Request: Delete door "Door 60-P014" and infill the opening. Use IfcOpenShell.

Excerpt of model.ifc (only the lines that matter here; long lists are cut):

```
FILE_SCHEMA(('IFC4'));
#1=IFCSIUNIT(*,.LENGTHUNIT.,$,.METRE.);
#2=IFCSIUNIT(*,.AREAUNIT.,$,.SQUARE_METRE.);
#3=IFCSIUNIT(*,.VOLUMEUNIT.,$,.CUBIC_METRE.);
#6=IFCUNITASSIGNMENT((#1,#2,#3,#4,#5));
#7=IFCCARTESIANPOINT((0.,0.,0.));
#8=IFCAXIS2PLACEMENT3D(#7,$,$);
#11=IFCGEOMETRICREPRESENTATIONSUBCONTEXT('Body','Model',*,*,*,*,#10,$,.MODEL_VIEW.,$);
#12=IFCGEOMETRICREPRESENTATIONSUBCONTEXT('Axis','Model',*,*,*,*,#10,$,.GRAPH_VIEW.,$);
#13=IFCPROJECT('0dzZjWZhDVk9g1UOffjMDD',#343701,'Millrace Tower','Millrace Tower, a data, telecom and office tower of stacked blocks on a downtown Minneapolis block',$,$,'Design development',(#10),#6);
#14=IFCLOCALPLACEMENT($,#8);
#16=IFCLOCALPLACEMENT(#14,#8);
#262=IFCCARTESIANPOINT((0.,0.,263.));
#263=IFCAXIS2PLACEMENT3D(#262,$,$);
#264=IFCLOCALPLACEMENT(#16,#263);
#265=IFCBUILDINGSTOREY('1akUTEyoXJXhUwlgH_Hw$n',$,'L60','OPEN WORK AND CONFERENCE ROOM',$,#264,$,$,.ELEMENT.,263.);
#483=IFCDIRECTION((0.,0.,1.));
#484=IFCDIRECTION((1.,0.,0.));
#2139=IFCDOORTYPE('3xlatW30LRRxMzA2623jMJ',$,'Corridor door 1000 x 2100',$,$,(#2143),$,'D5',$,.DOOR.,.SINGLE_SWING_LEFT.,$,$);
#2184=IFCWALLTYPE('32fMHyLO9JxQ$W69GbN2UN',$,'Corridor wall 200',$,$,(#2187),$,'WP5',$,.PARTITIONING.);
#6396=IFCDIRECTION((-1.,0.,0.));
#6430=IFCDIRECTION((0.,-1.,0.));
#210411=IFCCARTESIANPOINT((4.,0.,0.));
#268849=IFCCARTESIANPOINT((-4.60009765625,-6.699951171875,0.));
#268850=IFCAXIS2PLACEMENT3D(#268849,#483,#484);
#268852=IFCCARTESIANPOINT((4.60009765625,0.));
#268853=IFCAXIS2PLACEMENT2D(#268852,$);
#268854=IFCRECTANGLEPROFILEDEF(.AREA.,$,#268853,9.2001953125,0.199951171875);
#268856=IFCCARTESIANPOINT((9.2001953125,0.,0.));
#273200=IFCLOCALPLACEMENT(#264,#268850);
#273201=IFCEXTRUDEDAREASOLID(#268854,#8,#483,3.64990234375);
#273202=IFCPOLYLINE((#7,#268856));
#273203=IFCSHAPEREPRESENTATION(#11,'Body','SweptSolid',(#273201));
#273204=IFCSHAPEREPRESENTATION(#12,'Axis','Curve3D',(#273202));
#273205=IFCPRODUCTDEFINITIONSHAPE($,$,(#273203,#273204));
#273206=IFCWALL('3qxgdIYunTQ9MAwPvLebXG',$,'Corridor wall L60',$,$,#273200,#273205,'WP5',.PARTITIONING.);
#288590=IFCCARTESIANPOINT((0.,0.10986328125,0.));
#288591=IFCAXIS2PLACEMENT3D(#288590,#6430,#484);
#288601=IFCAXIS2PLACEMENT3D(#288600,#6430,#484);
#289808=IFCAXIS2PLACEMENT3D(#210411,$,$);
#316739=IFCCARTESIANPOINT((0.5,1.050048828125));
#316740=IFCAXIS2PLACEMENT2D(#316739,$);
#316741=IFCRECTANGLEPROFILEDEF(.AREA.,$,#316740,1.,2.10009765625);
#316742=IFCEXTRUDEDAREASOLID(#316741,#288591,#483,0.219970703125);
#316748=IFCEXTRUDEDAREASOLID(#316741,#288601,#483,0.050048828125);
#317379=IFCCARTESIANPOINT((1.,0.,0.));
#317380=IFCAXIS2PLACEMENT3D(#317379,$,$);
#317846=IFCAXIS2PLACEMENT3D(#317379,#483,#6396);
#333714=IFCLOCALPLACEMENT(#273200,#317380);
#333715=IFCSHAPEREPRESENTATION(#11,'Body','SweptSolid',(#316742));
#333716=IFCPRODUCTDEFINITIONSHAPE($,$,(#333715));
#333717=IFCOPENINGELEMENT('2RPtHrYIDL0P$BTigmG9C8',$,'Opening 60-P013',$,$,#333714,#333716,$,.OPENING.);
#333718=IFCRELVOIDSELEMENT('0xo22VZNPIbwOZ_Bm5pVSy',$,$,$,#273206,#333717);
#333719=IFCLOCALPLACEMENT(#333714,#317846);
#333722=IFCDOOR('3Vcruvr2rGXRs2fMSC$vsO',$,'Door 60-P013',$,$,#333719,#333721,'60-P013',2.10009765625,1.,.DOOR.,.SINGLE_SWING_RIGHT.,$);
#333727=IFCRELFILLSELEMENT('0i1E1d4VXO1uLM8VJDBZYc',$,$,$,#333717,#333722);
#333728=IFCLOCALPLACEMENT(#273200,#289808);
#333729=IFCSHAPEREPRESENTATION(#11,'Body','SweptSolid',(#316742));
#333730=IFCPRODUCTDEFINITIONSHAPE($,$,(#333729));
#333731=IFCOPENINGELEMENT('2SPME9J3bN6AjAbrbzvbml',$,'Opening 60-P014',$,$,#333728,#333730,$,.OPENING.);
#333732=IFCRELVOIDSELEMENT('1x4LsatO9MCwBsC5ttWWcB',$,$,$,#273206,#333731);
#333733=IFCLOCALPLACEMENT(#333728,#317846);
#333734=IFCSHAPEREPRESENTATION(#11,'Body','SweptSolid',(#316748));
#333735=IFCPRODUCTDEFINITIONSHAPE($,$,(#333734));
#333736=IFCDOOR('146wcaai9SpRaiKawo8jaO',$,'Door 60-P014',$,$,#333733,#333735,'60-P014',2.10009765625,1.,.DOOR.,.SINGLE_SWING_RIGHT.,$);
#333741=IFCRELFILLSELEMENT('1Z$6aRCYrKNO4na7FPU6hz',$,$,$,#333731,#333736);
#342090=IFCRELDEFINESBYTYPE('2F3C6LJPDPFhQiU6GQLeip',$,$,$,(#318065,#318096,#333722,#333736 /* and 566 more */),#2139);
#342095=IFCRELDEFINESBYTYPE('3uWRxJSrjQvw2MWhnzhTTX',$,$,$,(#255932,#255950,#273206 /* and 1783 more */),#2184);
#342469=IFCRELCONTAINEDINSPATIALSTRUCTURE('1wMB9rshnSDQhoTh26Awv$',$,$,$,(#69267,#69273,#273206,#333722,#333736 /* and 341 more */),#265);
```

```python
import ifcopenshell
import ifcopenshell.api.feature
import ifcopenshell.api.root
import ifcopenshell.geom
import ifcopenshell.util.shape

model = ifcopenshell.open("model.ifc")
settings = ifcopenshell.geom.settings()


def volume(element):
    """Net volume in cubic metres, openings subtracted."""
    shape = ifcopenshell.geom.create_shape(settings, element)
    return ifcopenshell.util.shape.get_volume(shape.geometry)


door = model.by_id(333736)
opening = door.FillsVoids[0].RelatingOpeningElement
wall = opening.VoidsElements[0].RelatingBuildingElement
before = volume(wall)

ifcopenshell.api.root.remove_product(model, product=door)
ifcopenshell.api.feature.remove_feature(model, feature=opening)

after = volume(wall)

print(f"wall volume {before:.3f} -> {after:.3f} m3")

model.write("model-out.ifc")
```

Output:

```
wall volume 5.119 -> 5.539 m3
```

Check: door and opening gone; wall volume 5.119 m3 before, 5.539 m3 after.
